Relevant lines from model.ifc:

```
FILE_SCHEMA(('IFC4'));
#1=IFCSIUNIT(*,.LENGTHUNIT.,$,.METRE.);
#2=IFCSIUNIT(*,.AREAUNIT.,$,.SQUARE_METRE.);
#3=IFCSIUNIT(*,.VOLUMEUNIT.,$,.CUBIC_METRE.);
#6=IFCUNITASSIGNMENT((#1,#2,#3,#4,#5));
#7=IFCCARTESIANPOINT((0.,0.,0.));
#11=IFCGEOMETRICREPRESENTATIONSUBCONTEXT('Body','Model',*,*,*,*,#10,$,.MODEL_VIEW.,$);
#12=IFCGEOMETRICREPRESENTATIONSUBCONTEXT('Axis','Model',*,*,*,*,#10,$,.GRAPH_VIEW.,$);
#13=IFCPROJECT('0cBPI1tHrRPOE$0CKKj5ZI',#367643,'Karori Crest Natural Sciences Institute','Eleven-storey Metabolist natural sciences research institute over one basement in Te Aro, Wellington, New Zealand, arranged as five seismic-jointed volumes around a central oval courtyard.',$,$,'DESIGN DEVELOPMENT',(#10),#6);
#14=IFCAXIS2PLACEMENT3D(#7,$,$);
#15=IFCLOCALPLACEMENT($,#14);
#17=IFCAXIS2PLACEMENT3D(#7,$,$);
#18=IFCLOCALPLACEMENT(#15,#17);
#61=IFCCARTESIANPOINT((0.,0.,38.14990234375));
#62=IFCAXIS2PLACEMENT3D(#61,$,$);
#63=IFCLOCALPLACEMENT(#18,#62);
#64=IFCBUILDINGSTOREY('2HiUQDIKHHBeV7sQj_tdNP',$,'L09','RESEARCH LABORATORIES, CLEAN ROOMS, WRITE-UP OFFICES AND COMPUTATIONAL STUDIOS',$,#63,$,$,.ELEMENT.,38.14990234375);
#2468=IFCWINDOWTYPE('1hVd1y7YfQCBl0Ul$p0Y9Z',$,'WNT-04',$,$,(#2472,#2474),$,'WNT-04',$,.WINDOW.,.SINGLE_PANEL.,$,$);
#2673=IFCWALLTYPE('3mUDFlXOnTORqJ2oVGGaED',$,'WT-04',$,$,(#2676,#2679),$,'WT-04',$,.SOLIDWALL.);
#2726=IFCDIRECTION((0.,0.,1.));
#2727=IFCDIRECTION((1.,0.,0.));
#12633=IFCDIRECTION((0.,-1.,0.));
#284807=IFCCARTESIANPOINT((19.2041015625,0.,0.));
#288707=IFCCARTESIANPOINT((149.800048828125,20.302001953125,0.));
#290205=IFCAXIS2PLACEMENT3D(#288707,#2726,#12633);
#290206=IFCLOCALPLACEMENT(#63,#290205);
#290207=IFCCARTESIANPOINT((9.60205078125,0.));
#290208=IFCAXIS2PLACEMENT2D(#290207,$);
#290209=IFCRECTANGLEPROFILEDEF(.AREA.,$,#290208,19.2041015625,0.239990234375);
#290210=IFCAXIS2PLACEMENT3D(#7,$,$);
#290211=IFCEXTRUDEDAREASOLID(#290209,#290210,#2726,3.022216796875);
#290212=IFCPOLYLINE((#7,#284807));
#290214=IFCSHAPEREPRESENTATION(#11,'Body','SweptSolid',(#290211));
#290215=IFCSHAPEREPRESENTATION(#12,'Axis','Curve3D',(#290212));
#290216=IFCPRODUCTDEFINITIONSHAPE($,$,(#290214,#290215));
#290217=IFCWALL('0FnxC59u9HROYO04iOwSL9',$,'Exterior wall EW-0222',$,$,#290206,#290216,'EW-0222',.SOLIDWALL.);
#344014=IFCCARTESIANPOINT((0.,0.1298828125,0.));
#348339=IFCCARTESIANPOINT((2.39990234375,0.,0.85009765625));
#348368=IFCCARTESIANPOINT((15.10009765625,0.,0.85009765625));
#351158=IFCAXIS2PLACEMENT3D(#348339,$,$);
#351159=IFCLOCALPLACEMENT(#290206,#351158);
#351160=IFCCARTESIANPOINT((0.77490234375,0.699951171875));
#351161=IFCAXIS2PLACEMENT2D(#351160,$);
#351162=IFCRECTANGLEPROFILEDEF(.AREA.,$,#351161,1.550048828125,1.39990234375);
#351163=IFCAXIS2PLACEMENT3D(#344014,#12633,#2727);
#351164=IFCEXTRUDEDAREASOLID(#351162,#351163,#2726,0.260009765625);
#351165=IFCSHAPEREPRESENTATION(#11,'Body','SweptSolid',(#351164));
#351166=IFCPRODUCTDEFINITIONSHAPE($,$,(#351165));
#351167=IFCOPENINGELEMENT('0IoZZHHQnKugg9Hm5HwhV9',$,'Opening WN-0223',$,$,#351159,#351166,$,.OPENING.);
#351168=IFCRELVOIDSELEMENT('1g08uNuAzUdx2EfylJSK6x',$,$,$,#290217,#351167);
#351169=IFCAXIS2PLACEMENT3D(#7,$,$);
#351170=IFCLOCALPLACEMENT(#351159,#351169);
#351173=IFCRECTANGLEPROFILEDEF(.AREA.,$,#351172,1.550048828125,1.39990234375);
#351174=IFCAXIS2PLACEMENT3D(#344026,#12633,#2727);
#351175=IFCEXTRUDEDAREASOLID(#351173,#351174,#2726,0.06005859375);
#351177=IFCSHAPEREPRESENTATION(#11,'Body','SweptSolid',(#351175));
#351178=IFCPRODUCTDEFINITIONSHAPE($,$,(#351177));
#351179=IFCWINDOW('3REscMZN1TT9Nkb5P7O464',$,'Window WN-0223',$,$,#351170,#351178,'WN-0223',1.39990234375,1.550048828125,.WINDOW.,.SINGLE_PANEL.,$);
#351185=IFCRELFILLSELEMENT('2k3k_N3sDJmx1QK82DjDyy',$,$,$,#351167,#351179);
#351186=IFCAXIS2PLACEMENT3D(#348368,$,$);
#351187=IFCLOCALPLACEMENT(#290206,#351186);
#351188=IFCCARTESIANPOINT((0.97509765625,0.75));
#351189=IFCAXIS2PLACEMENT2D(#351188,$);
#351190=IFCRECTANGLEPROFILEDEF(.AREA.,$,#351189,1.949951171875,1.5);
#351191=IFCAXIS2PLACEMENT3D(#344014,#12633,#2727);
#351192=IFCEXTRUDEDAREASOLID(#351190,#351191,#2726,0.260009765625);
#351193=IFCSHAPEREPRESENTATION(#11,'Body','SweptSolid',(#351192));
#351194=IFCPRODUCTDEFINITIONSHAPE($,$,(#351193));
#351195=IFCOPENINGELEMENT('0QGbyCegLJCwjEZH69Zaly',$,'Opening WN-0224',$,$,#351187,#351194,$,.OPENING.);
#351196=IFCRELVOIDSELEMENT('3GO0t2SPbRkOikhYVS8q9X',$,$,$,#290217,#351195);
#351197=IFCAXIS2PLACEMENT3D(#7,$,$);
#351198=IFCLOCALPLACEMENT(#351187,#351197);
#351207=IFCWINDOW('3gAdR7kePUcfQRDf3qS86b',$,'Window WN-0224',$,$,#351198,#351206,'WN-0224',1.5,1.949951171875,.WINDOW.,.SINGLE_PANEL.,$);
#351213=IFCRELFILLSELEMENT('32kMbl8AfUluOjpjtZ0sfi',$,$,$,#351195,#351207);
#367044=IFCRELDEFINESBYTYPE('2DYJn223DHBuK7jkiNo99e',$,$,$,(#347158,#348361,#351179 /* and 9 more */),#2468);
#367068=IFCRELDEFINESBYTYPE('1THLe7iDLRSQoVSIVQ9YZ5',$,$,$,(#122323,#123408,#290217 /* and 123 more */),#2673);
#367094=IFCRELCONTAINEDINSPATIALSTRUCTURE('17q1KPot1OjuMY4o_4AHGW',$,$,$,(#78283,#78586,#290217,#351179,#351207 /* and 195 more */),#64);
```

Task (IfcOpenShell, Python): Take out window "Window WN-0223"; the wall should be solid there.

```python
import ifcopenshell
import ifcopenshell.api.feature
import ifcopenshell.api.root
import ifcopenshell.geom
import ifcopenshell.util.shape

model = ifcopenshell.open("model.ifc")
settings = ifcopenshell.geom.settings()


def volume(element):
    """Net volume in cubic metres, openings subtracted."""
    shape = ifcopenshell.geom.create_shape(settings, element)
    return ifcopenshell.util.shape.get_volume(shape.geometry)


window = model.by_guid("3REscMZN1TT9Nkb5P7O464")
opening = window.FillsVoids[0].RelatingOpeningElement
wall = opening.VoidsElements[0].RelatingBuildingElement
before = volume(wall)

ifcopenshell.api.root.remove_product(model, product=window)
ifcopenshell.api.feature.remove_feature(model, feature=opening)

after = volume(wall)

print(f"wall volume {before:.3f} -> {after:.3f} m3")

model.write("model_v2.ifc")
```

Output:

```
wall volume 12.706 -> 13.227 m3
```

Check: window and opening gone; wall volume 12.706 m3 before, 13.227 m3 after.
